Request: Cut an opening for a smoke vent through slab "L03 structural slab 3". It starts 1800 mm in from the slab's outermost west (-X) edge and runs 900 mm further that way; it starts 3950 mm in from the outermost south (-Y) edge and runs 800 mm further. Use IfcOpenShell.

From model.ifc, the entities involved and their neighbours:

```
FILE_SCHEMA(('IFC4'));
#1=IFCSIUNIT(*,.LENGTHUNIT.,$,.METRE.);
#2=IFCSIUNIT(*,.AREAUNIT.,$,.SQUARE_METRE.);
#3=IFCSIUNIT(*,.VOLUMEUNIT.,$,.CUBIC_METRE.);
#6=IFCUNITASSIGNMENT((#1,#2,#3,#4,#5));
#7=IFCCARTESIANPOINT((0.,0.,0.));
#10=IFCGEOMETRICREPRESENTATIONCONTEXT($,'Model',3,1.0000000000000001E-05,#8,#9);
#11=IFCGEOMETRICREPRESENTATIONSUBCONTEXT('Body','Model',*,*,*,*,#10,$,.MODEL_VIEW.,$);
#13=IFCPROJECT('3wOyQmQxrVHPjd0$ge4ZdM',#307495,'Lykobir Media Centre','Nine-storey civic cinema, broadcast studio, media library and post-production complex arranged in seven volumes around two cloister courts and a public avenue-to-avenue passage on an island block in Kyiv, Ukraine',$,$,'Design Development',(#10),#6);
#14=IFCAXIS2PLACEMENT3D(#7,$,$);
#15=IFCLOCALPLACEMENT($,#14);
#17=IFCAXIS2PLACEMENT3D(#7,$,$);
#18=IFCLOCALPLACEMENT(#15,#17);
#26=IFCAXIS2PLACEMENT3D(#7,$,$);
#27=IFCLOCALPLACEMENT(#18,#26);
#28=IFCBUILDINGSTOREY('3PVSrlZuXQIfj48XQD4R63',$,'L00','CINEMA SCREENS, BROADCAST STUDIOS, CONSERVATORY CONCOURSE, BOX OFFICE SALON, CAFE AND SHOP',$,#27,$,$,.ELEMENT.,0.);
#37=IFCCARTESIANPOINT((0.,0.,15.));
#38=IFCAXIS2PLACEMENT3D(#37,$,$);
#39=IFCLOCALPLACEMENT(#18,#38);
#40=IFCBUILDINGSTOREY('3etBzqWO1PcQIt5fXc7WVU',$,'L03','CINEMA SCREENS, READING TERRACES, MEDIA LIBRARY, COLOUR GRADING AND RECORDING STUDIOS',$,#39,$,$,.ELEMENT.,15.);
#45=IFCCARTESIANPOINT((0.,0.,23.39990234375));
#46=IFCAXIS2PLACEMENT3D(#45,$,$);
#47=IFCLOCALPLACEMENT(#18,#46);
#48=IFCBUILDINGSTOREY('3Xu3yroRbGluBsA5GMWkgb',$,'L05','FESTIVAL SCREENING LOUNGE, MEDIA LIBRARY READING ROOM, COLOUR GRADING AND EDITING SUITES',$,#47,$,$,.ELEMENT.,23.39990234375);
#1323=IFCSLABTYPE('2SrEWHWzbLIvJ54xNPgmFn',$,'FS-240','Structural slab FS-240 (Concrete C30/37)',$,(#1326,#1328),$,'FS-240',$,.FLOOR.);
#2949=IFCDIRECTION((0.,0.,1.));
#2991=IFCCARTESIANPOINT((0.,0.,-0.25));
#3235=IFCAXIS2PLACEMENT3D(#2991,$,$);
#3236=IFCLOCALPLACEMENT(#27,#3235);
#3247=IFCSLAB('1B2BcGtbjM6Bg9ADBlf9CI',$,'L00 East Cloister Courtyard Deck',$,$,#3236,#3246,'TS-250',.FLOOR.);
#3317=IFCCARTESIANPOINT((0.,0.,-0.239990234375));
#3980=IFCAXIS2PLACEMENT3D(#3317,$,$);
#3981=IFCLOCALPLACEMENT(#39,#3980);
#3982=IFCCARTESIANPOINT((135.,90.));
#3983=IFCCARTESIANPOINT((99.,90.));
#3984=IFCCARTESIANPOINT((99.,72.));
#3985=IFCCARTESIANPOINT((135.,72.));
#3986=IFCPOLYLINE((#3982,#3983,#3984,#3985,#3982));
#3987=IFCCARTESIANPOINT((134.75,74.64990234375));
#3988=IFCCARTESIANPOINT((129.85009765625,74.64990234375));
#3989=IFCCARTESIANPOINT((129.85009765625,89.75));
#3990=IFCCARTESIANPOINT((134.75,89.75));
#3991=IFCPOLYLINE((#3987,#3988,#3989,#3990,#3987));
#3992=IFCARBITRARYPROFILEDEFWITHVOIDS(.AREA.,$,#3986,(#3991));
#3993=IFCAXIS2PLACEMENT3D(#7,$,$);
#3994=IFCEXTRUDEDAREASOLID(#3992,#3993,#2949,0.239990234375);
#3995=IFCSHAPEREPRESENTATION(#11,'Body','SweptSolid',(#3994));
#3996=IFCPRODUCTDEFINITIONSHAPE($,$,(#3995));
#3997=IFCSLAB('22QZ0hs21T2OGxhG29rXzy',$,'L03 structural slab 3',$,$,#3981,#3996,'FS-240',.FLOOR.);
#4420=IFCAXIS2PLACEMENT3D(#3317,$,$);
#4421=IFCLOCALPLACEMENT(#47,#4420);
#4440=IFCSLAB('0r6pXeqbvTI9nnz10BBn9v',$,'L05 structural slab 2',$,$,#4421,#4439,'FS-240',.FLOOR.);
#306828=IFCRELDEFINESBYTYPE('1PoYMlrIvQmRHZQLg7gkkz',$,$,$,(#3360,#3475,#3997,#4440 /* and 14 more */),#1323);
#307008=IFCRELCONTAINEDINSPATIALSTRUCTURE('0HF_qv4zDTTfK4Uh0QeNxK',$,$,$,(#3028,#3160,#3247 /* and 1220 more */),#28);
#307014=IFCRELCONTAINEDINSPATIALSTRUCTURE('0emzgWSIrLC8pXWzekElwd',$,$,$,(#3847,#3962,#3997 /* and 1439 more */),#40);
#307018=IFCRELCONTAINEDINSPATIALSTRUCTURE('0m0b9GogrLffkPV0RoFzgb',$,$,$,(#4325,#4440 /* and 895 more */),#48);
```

```python
import numpy as np
import ifcopenshell
import ifcopenshell.api.feature
import ifcopenshell.api.geometry
import ifcopenshell.api.root
import ifcopenshell.geom
import ifcopenshell.util.placement
import ifcopenshell.util.representation
import ifcopenshell.util.shape
import ifcopenshell.util.unit

model = ifcopenshell.open("model.ifc")
unit_scale = ifcopenshell.util.unit.calculate_unit_scale(model)
settings = ifcopenshell.geom.settings()


def volume(element):
    """Net volume in cubic metres, openings subtracted."""
    shape = ifcopenshell.geom.create_shape(settings, element)
    return ifcopenshell.util.shape.get_volume(shape.geometry)


slab = model.by_guid("22QZ0hs21T2OGxhG29rXzy")
before = volume(slab)

# Extent in the slab's own axes, in metres. The edges named are its -X and -Y sides.
slab_shape = ifcopenshell.geom.create_shape(settings, slab)
vertices = ifcopenshell.util.shape.get_vertices(slab_shape.geometry)
x_min, y_min, bottom = vertices.min(axis=0)
top = vertices[:, 2].max()

opening = ifcopenshell.api.root.create_entity(model, ifc_class="IfcOpeningElement", name="Smoke vent opening", predefined_type="OPENING")
context = ifcopenshell.util.representation.get_context(model, "Model", "Body", "MODEL_VIEW")
width, depth = 0.9, 0.8
outline = [(0.0, 0.0), (width, 0.0), (width, depth), (0.0, depth), (0.0, 0.0)]
# Overshoot both faces by 50 mm so the cut is clean.
shape = ifcopenshell.api.geometry.add_slab_representation(
    model, context=context, depth=top - bottom + 0.1, polyline=outline
)
ifcopenshell.api.geometry.assign_representation(model, product=opening, representation=shape)

matrix = ifcopenshell.util.placement.get_local_placement(slab.ObjectPlacement)
matrix[:, 3] = matrix @ np.append(np.array([x_min + 1.8, y_min + 3.95, bottom - 0.05]) / unit_scale, 1.0)
ifcopenshell.api.geometry.edit_object_placement(model, product=opening, matrix=matrix, is_si=False)
ifcopenshell.api.feature.add_feature(model, feature=opening, element=slab)

after = volume(slab)

print(f"slab volume {before:.3f} -> {after:.3f} m3")

model.write("model-out.ifc")
```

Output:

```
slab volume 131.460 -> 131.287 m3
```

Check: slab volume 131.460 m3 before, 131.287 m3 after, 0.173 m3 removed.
